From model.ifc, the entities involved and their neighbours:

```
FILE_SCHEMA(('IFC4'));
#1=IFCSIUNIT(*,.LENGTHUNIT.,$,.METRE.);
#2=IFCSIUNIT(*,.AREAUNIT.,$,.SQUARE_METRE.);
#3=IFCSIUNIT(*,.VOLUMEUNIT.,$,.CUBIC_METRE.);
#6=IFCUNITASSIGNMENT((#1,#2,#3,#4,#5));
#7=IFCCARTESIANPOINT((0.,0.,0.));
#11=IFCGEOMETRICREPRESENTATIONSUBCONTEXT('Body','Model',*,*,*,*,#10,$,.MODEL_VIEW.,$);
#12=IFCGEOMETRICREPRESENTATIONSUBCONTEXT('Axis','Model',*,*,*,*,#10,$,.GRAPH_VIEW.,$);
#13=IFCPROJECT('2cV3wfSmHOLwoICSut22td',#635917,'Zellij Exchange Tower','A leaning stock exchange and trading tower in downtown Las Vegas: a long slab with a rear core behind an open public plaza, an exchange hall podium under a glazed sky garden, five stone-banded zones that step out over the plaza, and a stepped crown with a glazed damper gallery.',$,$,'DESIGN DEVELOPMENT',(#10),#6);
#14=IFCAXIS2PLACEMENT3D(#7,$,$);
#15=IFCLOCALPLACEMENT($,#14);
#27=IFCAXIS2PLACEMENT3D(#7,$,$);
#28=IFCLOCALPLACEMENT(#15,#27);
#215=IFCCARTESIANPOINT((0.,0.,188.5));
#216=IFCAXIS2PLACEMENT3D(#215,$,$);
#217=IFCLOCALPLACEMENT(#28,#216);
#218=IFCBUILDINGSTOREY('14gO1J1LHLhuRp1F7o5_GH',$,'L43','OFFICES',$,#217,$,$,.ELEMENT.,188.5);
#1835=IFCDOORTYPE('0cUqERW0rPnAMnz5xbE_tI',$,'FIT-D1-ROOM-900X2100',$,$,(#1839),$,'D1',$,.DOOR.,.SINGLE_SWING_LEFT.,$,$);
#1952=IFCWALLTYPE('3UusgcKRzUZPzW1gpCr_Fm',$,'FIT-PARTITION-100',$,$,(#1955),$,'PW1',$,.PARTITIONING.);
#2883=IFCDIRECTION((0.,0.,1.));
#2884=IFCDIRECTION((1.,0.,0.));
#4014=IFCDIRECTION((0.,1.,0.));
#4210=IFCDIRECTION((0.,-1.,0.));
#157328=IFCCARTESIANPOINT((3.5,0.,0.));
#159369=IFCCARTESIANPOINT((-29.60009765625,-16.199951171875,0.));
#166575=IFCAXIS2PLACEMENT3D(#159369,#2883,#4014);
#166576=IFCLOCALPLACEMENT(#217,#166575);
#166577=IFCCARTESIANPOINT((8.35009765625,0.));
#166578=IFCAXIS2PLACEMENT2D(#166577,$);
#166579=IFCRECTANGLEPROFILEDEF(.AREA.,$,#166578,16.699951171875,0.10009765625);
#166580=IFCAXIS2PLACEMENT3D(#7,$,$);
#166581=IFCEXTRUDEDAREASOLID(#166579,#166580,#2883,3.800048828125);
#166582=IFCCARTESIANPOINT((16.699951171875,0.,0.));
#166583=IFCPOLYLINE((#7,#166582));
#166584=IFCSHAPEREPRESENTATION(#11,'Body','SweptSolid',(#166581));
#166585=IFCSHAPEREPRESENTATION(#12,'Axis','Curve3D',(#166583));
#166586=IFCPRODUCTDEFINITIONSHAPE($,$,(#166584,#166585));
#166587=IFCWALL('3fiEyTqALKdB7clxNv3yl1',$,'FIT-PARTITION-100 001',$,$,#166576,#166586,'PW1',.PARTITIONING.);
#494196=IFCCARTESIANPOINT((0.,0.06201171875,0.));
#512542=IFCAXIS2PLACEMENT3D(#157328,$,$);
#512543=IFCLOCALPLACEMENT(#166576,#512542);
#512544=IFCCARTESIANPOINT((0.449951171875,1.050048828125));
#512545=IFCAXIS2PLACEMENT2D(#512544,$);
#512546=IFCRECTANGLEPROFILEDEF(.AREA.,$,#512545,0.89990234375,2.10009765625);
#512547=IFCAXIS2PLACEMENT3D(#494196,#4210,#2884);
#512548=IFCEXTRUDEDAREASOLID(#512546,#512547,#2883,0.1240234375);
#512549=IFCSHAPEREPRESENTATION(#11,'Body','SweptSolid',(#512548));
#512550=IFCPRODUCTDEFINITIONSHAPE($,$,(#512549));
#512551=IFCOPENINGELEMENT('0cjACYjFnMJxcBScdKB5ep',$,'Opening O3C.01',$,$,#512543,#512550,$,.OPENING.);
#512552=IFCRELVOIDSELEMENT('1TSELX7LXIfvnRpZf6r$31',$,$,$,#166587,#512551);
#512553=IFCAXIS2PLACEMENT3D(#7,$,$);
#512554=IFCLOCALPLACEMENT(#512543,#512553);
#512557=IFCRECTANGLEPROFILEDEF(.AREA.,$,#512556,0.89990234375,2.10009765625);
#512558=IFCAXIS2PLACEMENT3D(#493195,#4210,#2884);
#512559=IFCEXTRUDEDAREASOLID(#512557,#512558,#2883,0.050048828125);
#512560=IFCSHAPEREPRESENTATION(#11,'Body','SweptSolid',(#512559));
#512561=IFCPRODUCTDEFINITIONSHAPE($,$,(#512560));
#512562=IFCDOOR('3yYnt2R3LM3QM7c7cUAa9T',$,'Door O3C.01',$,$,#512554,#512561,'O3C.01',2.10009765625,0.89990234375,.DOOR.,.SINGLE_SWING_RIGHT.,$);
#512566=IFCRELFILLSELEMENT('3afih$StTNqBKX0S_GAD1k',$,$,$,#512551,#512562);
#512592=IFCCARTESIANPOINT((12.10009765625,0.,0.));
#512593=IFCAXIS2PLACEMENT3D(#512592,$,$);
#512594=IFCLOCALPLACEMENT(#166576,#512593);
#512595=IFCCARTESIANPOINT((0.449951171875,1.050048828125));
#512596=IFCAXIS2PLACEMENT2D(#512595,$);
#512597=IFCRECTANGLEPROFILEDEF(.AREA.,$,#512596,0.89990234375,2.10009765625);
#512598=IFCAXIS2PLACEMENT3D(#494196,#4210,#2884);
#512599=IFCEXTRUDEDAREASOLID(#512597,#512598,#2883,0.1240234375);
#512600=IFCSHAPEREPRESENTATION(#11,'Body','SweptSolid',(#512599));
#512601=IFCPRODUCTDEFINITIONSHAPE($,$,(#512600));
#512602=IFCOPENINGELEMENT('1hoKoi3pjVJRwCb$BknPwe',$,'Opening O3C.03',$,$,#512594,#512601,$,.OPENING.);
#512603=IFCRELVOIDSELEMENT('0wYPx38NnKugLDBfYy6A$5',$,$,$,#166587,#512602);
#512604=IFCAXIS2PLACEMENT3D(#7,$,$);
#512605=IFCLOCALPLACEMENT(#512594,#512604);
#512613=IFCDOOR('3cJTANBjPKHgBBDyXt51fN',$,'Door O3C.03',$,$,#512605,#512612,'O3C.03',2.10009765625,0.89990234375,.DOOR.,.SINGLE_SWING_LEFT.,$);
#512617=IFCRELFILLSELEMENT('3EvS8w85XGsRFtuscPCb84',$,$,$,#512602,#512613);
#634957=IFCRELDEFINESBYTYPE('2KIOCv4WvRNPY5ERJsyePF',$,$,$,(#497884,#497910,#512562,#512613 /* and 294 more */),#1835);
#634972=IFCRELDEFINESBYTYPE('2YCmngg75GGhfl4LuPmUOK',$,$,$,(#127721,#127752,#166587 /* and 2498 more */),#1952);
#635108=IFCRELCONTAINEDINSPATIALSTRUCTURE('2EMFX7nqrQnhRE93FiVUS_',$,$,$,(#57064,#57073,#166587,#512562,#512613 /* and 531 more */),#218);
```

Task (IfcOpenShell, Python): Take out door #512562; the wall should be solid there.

```python
import ifcopenshell
import ifcopenshell.api.feature
import ifcopenshell.api.root
import ifcopenshell.geom
import ifcopenshell.util.shape

model = ifcopenshell.open("model.ifc")
settings = ifcopenshell.geom.settings()


def volume(element):
    """Net volume in cubic metres, openings subtracted."""
    shape = ifcopenshell.geom.create_shape(settings, element)
    return ifcopenshell.util.shape.get_volume(shape.geometry)


door = model.by_guid("3yYnt2R3LM3QM7c7cUAa9T")
opening = door.FillsVoids[0].RelatingOpeningElement
wall = opening.VoidsElements[0].RelatingBuildingElement
before = volume(wall)

ifcopenshell.api.root.remove_product(model, product=door)
ifcopenshell.api.feature.remove_feature(model, feature=opening)

after = volume(wall)

print(f"wall volume {before:.3f} -> {after:.3f} m3")

model.write("model_v2.ifc")
```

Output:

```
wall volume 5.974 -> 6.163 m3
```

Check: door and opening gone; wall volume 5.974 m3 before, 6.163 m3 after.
